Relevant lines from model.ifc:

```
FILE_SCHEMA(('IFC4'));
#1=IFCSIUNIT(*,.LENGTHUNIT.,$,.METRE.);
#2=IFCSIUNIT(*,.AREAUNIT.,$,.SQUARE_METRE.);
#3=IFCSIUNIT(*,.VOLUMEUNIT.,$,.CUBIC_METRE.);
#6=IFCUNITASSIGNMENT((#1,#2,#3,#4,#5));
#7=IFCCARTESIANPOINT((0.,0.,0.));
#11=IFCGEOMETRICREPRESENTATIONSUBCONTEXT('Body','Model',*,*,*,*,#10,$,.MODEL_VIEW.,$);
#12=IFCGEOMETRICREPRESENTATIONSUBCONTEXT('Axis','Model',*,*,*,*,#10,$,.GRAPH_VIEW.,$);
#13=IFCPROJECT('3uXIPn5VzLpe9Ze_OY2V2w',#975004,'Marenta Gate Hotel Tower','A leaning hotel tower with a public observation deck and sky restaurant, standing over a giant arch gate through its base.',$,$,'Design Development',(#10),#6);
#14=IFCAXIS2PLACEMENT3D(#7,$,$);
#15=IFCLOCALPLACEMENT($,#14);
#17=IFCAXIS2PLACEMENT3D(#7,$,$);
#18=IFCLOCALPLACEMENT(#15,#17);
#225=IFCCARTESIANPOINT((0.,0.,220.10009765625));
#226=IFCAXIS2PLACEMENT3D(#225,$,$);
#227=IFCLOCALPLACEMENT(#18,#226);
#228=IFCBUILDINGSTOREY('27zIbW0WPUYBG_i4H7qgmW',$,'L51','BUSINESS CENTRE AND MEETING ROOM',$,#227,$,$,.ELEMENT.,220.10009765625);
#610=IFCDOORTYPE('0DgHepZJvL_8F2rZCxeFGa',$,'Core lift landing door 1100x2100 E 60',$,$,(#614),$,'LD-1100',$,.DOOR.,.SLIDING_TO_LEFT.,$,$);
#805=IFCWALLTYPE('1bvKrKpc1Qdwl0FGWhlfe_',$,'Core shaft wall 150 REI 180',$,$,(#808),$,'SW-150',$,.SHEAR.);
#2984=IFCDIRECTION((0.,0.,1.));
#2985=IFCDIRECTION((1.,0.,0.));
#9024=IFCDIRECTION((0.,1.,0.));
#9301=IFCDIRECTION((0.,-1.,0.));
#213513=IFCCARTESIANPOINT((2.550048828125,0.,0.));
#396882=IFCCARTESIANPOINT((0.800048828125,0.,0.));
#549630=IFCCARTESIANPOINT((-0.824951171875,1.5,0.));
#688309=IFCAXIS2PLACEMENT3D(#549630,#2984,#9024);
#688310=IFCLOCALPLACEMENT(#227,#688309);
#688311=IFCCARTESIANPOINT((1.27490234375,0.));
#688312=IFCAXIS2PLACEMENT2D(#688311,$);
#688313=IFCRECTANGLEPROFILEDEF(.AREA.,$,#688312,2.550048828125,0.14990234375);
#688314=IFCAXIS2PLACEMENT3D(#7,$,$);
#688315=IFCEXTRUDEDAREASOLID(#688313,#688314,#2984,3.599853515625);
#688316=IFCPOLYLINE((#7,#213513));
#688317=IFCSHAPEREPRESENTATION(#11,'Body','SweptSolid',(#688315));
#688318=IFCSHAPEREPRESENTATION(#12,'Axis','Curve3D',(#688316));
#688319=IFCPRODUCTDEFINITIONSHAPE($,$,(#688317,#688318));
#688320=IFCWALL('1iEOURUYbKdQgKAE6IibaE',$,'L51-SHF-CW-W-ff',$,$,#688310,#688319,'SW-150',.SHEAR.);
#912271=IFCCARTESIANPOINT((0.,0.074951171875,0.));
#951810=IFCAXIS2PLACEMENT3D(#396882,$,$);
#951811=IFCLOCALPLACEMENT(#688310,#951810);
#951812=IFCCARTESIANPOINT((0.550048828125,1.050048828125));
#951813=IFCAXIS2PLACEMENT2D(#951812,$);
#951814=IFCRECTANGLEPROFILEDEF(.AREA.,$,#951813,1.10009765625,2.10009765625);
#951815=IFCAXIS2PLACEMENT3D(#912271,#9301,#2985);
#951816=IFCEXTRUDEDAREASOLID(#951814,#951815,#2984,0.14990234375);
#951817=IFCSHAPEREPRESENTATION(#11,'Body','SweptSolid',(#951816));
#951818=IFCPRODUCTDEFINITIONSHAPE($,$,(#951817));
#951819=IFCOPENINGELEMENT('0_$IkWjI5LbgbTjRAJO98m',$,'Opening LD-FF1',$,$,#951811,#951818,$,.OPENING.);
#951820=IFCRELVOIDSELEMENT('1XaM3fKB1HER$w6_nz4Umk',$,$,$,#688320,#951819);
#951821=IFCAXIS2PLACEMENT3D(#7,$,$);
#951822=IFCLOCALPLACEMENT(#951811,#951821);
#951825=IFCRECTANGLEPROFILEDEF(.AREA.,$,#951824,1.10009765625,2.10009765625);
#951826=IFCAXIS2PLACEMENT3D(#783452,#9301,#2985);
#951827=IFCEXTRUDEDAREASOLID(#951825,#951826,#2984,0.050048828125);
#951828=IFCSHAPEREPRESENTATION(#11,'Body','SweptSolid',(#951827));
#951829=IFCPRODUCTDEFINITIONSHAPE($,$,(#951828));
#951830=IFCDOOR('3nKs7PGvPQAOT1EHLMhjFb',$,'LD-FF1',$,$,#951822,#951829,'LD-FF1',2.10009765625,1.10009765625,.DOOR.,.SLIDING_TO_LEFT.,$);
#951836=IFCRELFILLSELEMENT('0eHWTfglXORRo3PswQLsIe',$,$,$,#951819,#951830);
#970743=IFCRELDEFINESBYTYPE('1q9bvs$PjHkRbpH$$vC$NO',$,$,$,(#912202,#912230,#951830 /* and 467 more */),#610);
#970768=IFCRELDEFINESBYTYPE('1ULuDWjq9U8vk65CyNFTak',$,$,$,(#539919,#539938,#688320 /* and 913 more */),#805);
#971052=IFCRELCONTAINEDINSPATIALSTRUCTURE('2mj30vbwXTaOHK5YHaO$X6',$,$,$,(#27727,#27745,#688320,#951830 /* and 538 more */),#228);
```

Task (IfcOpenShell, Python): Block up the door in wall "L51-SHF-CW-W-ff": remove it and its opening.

```python
import ifcopenshell
import ifcopenshell.api.feature
import ifcopenshell.api.root
import ifcopenshell.geom
import ifcopenshell.util.shape

model = ifcopenshell.open("model.ifc")
settings = ifcopenshell.geom.settings()


def volume(element):
    """Net volume in cubic metres, openings subtracted."""
    shape = ifcopenshell.geom.create_shape(settings, element)
    return ifcopenshell.util.shape.get_volume(shape.geometry)


door = model.by_guid("3nKs7PGvPQAOT1EHLMhjFb")
opening = door.FillsVoids[0].RelatingOpeningElement
wall = opening.VoidsElements[0].RelatingBuildingElement
before = volume(wall)

ifcopenshell.api.root.remove_product(model, product=door)
ifcopenshell.api.feature.remove_feature(model, feature=opening)

after = volume(wall)

print(f"wall volume {before:.3f} -> {after:.3f} m3")

model.write("model_edited.ifc")
```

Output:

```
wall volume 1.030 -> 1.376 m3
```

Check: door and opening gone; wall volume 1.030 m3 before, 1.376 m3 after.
